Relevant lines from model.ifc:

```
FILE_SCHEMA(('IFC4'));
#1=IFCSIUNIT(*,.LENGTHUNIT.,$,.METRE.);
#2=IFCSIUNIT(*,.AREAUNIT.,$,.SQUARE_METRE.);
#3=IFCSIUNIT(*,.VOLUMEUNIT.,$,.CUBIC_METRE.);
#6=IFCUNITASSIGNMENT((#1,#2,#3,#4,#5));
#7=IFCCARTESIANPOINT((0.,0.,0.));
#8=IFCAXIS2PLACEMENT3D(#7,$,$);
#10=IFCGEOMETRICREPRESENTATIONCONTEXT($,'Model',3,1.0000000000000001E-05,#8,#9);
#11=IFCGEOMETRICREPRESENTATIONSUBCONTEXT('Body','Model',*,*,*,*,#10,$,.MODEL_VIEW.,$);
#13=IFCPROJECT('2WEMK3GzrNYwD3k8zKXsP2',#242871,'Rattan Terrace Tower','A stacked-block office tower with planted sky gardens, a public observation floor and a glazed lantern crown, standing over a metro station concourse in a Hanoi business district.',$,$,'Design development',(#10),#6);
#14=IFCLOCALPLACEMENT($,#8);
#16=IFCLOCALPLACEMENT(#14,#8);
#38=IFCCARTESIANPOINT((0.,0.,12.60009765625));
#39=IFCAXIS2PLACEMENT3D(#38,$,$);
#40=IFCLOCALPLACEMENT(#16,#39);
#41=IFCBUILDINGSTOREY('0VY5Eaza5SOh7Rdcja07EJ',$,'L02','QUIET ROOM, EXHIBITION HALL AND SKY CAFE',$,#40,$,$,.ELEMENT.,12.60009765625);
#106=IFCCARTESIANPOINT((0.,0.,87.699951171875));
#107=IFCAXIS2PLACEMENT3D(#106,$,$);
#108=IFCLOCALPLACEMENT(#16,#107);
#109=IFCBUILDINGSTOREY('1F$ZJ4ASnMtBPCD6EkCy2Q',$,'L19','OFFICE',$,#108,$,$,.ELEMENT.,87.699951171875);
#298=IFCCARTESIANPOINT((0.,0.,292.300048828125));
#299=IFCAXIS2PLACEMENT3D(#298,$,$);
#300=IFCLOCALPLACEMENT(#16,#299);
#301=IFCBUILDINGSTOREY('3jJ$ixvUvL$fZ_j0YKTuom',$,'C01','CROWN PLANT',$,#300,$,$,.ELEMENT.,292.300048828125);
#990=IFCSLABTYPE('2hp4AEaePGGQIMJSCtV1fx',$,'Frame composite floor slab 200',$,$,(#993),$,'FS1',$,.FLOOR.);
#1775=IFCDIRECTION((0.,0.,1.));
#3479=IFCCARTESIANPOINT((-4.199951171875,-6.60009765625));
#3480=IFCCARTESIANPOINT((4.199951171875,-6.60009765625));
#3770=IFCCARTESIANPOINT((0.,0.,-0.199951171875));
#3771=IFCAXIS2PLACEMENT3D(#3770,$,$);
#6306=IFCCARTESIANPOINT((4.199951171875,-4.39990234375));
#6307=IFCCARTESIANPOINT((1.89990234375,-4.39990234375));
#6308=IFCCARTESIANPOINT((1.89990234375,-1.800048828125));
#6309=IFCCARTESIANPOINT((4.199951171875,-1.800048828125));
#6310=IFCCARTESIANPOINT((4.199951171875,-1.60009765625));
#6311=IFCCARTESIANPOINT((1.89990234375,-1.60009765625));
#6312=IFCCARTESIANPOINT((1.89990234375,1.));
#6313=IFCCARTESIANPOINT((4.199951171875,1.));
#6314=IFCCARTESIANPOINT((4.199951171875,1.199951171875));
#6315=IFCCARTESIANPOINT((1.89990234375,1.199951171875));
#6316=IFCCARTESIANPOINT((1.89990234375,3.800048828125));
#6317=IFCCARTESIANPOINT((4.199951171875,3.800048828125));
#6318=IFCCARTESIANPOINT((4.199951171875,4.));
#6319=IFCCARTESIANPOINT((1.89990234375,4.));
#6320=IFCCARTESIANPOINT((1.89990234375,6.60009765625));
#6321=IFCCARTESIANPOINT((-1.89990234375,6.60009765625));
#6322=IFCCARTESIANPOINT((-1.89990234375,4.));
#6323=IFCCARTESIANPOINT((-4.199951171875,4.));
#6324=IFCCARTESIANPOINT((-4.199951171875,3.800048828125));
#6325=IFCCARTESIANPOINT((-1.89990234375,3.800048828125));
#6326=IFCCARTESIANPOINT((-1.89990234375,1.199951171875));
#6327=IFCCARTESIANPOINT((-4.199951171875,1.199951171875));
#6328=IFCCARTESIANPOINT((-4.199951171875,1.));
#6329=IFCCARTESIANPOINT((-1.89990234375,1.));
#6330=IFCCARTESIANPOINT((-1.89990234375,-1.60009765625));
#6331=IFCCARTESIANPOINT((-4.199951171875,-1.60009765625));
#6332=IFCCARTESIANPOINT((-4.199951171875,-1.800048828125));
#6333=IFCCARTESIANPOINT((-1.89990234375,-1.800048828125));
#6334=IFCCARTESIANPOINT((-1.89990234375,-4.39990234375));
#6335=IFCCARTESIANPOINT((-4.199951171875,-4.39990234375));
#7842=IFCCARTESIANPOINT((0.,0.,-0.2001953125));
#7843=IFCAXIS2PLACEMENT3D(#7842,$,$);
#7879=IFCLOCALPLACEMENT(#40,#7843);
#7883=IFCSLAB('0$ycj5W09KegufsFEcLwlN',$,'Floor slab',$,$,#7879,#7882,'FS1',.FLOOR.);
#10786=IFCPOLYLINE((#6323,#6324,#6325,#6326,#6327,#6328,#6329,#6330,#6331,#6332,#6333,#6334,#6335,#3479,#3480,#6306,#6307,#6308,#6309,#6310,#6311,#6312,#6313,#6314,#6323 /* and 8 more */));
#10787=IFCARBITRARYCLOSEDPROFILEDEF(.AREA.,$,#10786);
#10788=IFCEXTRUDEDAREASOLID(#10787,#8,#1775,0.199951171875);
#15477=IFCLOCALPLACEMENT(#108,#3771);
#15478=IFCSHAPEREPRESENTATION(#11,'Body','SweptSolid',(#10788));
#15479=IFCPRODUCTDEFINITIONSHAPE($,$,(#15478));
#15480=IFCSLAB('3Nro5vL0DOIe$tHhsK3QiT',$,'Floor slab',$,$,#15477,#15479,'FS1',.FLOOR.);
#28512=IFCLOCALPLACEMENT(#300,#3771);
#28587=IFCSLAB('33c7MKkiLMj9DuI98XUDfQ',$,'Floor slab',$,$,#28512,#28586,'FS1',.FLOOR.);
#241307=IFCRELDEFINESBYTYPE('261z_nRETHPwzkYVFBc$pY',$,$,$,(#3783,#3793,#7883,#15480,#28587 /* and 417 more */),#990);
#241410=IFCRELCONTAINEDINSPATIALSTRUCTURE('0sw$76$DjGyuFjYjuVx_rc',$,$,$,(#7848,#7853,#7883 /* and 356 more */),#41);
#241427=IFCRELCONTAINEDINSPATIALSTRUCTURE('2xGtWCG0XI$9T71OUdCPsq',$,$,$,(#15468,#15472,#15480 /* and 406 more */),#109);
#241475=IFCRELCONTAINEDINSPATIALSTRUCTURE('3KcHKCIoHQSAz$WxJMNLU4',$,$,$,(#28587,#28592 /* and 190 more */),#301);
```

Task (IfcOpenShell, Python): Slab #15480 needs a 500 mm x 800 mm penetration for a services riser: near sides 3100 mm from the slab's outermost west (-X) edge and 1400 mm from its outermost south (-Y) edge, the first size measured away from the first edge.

```python
import numpy as np
import ifcopenshell
import ifcopenshell.api.feature
import ifcopenshell.api.geometry
import ifcopenshell.api.root
import ifcopenshell.geom
import ifcopenshell.util.placement
import ifcopenshell.util.representation
import ifcopenshell.util.shape
import ifcopenshell.util.unit

model = ifcopenshell.open("model.ifc")
unit_scale = ifcopenshell.util.unit.calculate_unit_scale(model)
settings = ifcopenshell.geom.settings()


def volume(element):
    """Net volume in cubic metres, openings subtracted."""
    shape = ifcopenshell.geom.create_shape(settings, element)
    return ifcopenshell.util.shape.get_volume(shape.geometry)


slab = model.by_id(15480)
before = volume(slab)

# Extent in the slab's own axes, in metres. The edges named are its -X and -Y sides.
slab_shape = ifcopenshell.geom.create_shape(settings, slab)
vertices = ifcopenshell.util.shape.get_vertices(slab_shape.geometry)
x_min, y_min, bottom = vertices.min(axis=0)
top = vertices[:, 2].max()

opening = ifcopenshell.api.root.create_entity(model, ifc_class="IfcOpeningElement", name="Services riser opening", predefined_type="OPENING")
context = ifcopenshell.util.representation.get_context(model, "Model", "Body", "MODEL_VIEW")
width, depth = 0.5, 0.8
outline = [(0.0, 0.0), (width, 0.0), (width, depth), (0.0, depth), (0.0, 0.0)]
# Overshoot both faces by 50 mm so the cut is clean.
shape = ifcopenshell.api.geometry.add_slab_representation(
    model, context=context, depth=top - bottom + 0.1, polyline=outline
)
ifcopenshell.api.geometry.assign_representation(model, product=opening, representation=shape)

matrix = ifcopenshell.util.placement.get_local_placement(slab.ObjectPlacement)
matrix[:, 3] = matrix @ np.append(np.array([x_min + 3.1, y_min + 1.4, bottom - 0.05]) / unit_scale, 1.0)
ifcopenshell.api.geometry.edit_object_placement(model, product=opening, matrix=matrix, is_si=False)
ifcopenshell.api.feature.add_feature(model, feature=opening, element=slab)

after = volume(slab)

print(f"slab volume {before:.3f} -> {after:.3f} m3")

model.write("model-out.ifc")
```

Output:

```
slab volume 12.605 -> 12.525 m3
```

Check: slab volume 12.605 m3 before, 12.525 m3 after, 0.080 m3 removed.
